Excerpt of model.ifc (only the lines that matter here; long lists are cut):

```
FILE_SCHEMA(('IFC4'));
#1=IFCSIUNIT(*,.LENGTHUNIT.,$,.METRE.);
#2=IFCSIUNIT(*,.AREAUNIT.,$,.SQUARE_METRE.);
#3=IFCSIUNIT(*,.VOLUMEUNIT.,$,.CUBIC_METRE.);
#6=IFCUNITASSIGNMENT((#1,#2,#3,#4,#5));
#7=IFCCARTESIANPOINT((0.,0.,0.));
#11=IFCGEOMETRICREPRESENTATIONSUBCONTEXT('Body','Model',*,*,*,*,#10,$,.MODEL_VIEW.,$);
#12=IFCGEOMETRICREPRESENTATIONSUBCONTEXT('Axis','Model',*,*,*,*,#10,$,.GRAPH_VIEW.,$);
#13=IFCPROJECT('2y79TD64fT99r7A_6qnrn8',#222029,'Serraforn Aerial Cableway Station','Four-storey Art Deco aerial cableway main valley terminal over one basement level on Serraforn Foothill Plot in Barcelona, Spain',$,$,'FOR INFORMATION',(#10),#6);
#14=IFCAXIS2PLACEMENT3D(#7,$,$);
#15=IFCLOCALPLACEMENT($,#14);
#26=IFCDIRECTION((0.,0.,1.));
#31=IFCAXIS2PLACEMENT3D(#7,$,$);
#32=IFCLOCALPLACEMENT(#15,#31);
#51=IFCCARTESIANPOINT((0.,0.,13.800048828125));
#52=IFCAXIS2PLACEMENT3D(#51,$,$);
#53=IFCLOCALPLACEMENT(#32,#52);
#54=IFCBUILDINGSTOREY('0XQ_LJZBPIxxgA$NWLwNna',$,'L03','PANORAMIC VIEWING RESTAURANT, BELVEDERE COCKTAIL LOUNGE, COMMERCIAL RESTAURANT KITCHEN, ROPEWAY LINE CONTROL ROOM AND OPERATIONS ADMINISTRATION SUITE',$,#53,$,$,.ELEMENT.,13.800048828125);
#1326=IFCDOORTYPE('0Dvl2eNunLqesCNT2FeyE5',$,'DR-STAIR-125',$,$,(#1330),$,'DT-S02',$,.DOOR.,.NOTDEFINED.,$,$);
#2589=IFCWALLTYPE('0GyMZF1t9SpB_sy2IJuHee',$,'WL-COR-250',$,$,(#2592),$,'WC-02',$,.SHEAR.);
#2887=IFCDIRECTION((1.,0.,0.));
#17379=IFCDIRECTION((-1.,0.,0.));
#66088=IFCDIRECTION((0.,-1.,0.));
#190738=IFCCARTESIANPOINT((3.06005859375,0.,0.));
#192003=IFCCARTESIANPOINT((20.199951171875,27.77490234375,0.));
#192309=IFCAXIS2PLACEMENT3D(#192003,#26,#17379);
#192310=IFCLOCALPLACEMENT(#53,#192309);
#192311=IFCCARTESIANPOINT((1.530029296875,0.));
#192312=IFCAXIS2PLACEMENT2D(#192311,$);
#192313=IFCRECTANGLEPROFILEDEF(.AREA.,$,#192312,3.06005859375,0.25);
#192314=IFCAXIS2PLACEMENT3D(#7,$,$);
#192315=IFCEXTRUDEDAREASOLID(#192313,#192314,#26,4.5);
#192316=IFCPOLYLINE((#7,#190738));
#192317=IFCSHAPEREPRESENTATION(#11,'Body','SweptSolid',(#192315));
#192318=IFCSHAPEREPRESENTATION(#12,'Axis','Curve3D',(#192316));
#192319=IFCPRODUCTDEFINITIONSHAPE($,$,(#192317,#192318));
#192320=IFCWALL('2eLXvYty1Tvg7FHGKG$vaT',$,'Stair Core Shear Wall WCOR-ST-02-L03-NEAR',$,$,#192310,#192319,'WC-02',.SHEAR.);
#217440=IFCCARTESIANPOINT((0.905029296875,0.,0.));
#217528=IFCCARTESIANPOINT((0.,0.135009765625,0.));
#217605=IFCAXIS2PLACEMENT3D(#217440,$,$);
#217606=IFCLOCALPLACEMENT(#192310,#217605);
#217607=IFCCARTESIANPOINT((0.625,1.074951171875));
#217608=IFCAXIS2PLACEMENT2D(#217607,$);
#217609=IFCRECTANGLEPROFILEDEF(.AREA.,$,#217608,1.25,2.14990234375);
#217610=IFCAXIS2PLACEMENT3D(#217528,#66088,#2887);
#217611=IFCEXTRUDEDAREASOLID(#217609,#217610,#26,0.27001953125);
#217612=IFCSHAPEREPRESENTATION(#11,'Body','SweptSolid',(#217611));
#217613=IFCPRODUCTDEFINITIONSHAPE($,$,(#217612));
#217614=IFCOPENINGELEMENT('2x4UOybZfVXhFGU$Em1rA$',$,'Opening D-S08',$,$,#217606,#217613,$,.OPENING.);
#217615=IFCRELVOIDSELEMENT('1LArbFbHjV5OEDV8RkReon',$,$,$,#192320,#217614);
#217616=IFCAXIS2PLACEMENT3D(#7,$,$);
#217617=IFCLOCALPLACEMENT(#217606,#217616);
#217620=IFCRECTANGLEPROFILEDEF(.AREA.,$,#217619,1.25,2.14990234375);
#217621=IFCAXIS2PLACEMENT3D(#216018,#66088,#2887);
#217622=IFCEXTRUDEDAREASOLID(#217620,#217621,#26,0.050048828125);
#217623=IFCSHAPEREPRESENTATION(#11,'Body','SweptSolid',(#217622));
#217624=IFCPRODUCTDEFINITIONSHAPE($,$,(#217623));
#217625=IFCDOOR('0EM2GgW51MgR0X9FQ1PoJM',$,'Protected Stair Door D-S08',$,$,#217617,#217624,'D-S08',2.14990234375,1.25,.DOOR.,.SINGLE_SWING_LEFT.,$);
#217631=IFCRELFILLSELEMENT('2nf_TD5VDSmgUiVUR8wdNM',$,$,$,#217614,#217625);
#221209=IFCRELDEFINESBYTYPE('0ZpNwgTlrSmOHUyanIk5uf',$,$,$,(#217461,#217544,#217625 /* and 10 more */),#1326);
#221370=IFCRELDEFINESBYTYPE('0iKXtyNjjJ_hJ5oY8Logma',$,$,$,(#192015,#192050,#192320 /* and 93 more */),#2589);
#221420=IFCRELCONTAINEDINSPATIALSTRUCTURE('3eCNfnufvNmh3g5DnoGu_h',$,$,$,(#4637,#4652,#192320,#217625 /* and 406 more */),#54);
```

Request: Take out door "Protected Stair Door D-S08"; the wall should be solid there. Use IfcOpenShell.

```python
import ifcopenshell
import ifcopenshell.api.feature
import ifcopenshell.api.root
import ifcopenshell.geom
import ifcopenshell.util.shape

model = ifcopenshell.open("model.ifc")
settings = ifcopenshell.geom.settings()


def volume(element):
    """Net volume in cubic metres, openings subtracted."""
    shape = ifcopenshell.geom.create_shape(settings, element)
    return ifcopenshell.util.shape.get_volume(shape.geometry)


door = model.by_id(217625)
opening = door.FillsVoids[0].RelatingOpeningElement
wall = opening.VoidsElements[0].RelatingBuildingElement
before = volume(wall)

ifcopenshell.api.root.remove_product(model, product=door)
ifcopenshell.api.feature.remove_feature(model, feature=opening)

after = volume(wall)

print(f"wall volume {before:.3f} -> {after:.3f} m3")

model.write("model_v2.ifc")
```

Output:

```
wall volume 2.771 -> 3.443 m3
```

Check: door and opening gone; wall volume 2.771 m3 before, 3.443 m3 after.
